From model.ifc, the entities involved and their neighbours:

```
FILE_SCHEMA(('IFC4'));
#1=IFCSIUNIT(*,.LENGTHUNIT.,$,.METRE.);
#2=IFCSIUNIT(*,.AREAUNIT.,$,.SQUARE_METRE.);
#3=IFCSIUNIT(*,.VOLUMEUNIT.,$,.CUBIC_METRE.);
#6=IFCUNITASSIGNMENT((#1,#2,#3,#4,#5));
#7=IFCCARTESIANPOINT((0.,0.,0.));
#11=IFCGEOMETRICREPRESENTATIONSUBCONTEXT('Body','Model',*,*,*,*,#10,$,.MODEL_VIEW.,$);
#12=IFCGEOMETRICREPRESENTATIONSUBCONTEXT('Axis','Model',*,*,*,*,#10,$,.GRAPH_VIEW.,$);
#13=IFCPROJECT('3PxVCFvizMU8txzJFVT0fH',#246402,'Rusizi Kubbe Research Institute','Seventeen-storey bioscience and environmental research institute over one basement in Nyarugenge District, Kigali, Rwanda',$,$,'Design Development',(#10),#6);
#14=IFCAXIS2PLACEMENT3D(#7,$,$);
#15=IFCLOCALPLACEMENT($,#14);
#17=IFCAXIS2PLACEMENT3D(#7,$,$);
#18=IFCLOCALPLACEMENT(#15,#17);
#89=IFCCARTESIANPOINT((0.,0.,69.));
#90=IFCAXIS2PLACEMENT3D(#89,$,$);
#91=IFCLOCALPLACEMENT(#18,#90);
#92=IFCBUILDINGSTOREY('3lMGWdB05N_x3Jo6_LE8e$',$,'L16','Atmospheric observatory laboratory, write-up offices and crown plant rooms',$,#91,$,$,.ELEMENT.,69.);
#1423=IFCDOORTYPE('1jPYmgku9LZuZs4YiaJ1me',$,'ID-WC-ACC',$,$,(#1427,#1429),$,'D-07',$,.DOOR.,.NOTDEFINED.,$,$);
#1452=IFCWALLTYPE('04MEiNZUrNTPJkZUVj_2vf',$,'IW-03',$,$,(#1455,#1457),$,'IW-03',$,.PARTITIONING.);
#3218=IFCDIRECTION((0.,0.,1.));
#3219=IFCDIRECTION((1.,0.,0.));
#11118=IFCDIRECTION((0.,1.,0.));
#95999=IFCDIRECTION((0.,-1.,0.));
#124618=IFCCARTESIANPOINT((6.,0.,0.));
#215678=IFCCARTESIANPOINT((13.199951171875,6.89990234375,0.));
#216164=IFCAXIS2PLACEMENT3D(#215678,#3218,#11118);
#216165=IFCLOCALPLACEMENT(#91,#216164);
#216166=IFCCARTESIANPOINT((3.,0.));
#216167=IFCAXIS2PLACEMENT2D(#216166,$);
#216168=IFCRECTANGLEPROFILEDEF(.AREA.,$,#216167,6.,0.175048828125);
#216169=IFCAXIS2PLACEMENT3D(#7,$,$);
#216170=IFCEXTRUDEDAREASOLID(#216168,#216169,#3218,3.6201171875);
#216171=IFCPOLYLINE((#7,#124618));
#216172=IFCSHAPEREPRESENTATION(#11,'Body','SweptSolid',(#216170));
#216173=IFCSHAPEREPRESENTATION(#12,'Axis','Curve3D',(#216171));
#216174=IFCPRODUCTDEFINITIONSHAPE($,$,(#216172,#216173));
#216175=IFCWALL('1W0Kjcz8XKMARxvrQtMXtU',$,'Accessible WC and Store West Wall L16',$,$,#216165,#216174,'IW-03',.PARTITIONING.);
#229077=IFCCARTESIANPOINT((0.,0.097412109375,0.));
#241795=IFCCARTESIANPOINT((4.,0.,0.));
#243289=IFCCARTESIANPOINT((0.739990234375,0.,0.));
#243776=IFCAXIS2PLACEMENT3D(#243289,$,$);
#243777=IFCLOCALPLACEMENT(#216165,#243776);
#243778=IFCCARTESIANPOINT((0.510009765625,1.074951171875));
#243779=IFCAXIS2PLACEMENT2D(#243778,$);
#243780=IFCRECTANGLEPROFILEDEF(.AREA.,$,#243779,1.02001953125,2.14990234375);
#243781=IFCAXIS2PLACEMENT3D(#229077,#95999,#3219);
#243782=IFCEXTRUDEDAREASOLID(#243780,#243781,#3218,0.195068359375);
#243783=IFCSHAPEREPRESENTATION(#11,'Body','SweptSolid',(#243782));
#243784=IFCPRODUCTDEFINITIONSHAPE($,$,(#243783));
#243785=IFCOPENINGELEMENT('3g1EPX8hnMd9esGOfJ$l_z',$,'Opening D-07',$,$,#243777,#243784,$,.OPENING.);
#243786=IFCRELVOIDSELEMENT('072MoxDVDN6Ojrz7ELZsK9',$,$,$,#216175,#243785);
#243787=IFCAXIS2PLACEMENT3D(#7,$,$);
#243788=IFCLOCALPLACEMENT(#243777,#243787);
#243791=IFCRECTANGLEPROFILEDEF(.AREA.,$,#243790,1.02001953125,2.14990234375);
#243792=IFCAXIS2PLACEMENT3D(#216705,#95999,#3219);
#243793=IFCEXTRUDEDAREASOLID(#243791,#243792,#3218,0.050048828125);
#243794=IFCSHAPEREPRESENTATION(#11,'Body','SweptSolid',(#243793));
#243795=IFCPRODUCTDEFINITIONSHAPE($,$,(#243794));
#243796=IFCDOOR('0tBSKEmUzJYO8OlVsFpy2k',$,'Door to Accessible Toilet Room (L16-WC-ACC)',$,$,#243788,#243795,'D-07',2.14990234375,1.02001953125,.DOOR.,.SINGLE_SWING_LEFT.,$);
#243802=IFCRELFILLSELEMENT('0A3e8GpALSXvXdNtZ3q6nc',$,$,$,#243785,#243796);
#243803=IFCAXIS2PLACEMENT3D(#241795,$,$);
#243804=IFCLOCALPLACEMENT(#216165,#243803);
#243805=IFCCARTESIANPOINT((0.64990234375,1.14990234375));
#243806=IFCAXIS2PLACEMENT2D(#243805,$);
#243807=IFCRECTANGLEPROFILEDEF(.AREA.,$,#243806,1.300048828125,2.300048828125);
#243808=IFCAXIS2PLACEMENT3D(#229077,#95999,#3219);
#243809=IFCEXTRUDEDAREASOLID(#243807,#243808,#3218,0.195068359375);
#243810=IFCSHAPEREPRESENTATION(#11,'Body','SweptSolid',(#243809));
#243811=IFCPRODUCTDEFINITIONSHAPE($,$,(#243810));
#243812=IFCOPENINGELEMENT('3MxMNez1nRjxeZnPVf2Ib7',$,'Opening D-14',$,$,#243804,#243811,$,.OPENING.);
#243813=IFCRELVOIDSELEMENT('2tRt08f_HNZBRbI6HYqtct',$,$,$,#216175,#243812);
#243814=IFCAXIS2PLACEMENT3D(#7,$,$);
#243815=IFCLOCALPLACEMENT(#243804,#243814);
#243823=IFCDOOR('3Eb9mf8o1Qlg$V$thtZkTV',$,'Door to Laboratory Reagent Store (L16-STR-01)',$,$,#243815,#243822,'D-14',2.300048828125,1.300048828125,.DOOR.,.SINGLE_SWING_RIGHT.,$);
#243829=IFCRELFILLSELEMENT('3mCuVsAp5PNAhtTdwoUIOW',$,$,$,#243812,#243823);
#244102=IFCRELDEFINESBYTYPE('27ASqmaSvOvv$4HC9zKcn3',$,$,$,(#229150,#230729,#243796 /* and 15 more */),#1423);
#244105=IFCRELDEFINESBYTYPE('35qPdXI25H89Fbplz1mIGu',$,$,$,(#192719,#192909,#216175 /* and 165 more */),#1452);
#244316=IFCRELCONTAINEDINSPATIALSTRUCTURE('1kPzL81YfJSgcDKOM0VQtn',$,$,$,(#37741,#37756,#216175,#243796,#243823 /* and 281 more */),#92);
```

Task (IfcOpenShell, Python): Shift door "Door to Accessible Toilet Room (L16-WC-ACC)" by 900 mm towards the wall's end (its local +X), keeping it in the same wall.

```python
import ifcopenshell
import ifcopenshell.api.geometry
import ifcopenshell.util.placement

model = ifcopenshell.open("model.ifc")

door = model.by_id(243796)
opening = door.FillsVoids[0].RelatingOpeningElement
wall = opening.VoidsElements[0].RelatingBuildingElement

wall_matrix = ifcopenshell.util.placement.get_local_placement(wall.ObjectPlacement)
shift = wall_matrix[:3, 0] * 0.9
before = ifcopenshell.util.placement.get_local_placement(door.ObjectPlacement)[:3, 3].copy()

# The door is placed relative to its opening, so it follows when the opening moves.
matrix = ifcopenshell.util.placement.get_local_placement(opening.ObjectPlacement)
matrix[:3, 3] += shift
ifcopenshell.api.geometry.edit_object_placement(
    model, product=opening, matrix=matrix, is_si=False, should_transform_children=True
)

after = ifcopenshell.util.placement.get_local_placement(door.ObjectPlacement)[:3, 3]
print("door moved by", (after - before).round(3) + 0.0)

model.write("model-out.ifc")
```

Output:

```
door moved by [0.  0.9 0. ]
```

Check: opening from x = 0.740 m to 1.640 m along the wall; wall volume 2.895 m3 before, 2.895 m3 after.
